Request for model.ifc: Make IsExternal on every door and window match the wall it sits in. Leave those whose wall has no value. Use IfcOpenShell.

First a look at what the model holds.

```python
import ifcopenshell
import ifcopenshell.util.element

model = ifcopenshell.open("model.ifc")
print(model.schema)
seen = {}
for e in model.by_type("IfcDoor") + model.by_type("IfcWindow"):
    if not e.FillsVoids:
        continue
    host = e.FillsVoids[0].RelatingOpeningElement.VoidsElements[0].RelatingBuildingElement
    own = ifcopenshell.util.element.get_pset(e, f"Pset_{e.is_a()[3:].removesuffix('StandardCase')}Common", "IsExternal")
    wall = ifcopenshell.util.element.get_pset(host, "Pset_WallCommon", "IsExternal")
    seen[e.is_a(), own, wall] = seen.get((e.is_a(), own, wall), 0) + 1
for (cls, own, wall), count in sorted(seen.items(), key=str):
    print(count, cls, "IsExternal:", own, "| host wall:", wall)
```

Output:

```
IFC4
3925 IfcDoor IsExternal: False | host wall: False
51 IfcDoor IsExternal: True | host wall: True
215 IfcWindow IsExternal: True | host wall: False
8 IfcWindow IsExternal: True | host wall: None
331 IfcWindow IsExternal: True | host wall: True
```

```python
import ifcopenshell
import ifcopenshell.api.pset
import ifcopenshell.util.element

model = ifcopenshell.open("model.ifc")

count = 0
for ifc_class, pset_name in (("IfcDoor", "Pset_DoorCommon"), ("IfcWindow", "Pset_WindowCommon")):
    for e in model.by_type(ifc_class):
        if not e.FillsVoids:
            continue
        host = e.FillsVoids[0].RelatingOpeningElement.VoidsElements[0].RelatingBuildingElement
        external = ifcopenshell.util.element.get_pset(host, "Pset_WallCommon", "IsExternal")
        if external is None or ifcopenshell.util.element.get_pset(e, pset_name, "IsExternal") == external:
            continue
        found = ifcopenshell.util.element.get_pset(e, pset_name, should_inherit=False)
        if found:
            pset = model.by_id(found["id"])
            if len(ifcopenshell.util.element.get_elements_by_pset(pset)) > 1:
                pset = ifcopenshell.api.pset.unshare_pset(model, products=[e], pset=pset)[0]
        else:
            pset = ifcopenshell.api.pset.add_pset(model, product=e, name=pset_name)
        ifcopenshell.api.pset.edit_pset(model, pset=pset, properties={"IsExternal": external})
        count += 1

print(count, "updated")

model.write("model_rev.ifc")
```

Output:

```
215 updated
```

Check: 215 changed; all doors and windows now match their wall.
